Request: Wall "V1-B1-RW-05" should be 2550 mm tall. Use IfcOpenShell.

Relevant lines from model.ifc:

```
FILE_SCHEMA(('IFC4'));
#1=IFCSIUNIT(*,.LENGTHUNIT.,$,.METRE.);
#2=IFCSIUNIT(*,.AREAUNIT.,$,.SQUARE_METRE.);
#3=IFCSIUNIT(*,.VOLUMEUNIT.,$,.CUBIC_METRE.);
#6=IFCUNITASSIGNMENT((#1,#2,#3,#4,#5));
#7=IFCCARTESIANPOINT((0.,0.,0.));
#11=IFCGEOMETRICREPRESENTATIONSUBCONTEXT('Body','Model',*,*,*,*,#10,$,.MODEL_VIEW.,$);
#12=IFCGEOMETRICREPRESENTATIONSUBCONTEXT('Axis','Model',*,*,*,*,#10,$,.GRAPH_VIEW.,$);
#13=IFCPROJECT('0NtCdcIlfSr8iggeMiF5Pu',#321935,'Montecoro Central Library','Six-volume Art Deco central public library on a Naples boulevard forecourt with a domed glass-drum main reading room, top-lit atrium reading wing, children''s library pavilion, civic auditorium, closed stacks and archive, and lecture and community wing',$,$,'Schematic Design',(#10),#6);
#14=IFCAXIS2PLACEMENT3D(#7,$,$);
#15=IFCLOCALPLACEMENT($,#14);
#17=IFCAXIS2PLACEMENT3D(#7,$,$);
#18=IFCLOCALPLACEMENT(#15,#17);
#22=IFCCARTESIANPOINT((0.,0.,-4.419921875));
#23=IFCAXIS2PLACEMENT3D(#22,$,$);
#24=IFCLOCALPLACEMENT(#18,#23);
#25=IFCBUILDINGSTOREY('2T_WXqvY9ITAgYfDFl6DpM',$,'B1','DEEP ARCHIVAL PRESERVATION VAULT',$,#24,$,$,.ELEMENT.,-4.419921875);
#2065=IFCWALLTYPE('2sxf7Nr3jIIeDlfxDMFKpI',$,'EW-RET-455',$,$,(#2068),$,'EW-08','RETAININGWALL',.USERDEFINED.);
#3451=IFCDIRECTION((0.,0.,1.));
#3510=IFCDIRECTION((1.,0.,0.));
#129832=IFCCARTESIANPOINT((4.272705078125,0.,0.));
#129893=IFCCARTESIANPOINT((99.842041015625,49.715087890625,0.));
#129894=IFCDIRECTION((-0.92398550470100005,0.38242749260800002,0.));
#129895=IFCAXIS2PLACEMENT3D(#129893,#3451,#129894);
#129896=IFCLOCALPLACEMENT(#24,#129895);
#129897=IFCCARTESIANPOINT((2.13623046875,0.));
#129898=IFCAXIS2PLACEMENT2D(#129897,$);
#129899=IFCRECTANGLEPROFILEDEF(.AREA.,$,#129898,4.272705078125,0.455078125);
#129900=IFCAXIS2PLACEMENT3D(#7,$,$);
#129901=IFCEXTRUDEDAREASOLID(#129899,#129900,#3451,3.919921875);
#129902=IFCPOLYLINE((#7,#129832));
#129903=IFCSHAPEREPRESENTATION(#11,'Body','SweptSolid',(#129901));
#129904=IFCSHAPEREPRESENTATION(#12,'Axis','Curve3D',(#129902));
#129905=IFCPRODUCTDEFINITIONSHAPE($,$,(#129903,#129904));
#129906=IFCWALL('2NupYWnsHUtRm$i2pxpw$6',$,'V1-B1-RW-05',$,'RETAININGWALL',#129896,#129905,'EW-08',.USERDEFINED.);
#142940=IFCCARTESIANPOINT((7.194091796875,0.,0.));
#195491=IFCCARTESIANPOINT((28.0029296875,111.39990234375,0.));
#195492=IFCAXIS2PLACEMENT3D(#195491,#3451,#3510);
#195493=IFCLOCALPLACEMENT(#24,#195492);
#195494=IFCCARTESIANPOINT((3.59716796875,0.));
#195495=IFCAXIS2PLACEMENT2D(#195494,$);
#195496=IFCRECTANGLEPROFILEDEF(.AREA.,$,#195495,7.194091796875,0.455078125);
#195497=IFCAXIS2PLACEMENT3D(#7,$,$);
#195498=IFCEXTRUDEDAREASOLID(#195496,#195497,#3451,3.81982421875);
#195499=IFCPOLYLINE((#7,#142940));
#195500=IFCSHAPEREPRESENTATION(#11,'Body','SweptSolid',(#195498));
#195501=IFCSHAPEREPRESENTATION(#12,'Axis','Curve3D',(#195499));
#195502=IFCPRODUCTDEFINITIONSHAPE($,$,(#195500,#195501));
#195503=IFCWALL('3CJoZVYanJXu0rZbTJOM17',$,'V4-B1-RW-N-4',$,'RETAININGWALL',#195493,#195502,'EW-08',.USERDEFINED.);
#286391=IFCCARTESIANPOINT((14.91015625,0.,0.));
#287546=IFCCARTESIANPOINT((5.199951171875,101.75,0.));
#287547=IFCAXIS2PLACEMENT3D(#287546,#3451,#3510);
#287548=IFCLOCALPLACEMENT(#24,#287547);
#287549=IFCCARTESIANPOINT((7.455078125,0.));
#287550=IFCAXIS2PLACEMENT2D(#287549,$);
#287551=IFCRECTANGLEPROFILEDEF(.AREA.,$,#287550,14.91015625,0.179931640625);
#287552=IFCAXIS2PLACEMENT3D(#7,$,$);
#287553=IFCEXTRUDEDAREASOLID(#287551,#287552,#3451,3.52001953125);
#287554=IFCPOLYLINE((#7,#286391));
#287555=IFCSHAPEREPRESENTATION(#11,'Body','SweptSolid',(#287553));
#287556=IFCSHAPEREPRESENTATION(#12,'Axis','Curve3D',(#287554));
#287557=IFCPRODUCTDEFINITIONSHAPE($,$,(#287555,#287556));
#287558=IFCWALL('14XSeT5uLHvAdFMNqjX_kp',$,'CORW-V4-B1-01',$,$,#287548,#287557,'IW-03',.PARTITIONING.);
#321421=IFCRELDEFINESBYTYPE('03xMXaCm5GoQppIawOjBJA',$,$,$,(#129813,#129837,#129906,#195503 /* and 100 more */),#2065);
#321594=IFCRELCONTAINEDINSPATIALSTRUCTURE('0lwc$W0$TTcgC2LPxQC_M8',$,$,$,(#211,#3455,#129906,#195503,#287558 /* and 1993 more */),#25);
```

```python
import ifcopenshell
import ifcopenshell.geom
import ifcopenshell.util.representation
import ifcopenshell.util.shape
import ifcopenshell.util.unit

model = ifcopenshell.open("model.ifc")
unit_scale = ifcopenshell.util.unit.calculate_unit_scale(model)
settings = ifcopenshell.geom.settings()


def volume(element):
    """Net volume in cubic metres, openings subtracted."""
    shape = ifcopenshell.geom.create_shape(settings, element)
    return ifcopenshell.util.shape.get_volume(shape.geometry)


wall = model.by_guid("2NupYWnsHUtRm$i2pxpw$6")
before = volume(wall)

body = ifcopenshell.util.representation.get_representation(wall, "Model", "Body")
solid = body.Items[0]
old_height = solid.Depth
solid.Depth = 2.55 / unit_scale
after = volume(wall)

print(f"height {old_height:g} -> {solid.Depth:g}, volume {before:.3f} -> {after:.3f} m3")

model.write("model_v2.ifc")
```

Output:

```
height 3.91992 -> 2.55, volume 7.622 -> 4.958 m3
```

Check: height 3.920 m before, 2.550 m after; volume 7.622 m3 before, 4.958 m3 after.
